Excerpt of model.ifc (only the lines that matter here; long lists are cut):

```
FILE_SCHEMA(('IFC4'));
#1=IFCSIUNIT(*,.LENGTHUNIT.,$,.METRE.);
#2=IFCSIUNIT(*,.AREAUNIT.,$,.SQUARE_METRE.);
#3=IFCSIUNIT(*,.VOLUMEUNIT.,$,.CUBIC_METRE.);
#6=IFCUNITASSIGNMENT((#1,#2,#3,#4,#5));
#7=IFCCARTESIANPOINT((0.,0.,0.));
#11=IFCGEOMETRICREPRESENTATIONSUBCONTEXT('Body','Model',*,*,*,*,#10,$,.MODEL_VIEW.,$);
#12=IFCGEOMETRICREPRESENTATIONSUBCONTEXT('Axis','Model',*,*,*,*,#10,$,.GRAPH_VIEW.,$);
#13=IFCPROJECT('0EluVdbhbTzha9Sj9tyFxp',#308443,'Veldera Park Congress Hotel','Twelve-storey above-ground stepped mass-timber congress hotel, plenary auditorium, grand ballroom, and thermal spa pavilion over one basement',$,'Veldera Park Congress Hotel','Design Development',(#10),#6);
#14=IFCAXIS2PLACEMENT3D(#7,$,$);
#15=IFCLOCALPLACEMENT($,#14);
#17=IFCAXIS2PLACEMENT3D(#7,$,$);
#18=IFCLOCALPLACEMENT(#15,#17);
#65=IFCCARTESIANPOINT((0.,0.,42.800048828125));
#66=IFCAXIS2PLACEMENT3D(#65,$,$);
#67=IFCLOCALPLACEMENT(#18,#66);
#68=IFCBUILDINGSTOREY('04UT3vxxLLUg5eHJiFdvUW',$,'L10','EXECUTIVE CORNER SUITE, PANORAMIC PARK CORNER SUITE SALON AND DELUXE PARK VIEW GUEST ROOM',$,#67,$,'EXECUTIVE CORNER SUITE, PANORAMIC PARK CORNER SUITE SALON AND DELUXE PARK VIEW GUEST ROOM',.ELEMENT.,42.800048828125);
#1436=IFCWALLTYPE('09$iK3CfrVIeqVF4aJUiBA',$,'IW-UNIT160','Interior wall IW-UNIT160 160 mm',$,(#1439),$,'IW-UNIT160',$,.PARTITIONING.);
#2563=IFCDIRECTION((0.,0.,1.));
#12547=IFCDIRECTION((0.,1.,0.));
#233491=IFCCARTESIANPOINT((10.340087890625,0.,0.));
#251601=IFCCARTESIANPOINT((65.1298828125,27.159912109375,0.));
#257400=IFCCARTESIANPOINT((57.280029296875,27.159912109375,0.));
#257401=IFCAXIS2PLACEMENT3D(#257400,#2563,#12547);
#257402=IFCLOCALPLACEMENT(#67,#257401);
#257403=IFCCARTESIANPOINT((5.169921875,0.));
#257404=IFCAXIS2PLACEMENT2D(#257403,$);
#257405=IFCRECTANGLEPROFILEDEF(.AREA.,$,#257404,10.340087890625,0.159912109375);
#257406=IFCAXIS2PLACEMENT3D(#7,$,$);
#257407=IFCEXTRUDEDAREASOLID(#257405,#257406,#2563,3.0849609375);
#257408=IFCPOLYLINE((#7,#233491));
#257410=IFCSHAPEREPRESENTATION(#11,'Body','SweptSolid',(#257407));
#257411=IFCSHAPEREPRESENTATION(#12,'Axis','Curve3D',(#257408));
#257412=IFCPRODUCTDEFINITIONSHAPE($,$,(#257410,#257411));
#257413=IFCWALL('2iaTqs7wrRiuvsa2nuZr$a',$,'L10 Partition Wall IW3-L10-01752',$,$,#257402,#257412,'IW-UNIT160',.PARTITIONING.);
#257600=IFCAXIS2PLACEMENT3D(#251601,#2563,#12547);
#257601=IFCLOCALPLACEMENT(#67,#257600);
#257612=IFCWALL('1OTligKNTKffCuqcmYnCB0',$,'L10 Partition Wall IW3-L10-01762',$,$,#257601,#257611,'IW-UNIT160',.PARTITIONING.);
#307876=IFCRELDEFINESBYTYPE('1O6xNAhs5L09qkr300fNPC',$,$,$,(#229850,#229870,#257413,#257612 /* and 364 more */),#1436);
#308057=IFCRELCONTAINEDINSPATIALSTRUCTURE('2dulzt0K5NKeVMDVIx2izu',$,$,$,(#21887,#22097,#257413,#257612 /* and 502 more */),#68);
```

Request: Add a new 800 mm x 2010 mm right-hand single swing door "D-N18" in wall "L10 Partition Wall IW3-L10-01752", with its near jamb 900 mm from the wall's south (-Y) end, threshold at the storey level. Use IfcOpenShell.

```python
import numpy as np
import ifcopenshell
import ifcopenshell.api.feature
import ifcopenshell.api.geometry
import ifcopenshell.api.root
import ifcopenshell.api.spatial
import ifcopenshell.geom
import ifcopenshell.util.element
import ifcopenshell.util.placement
import ifcopenshell.util.representation
import ifcopenshell.util.shape
import ifcopenshell.util.unit

model = ifcopenshell.open("model.ifc")
unit_scale = ifcopenshell.util.unit.calculate_unit_scale(model)
settings = ifcopenshell.geom.settings()


def volume(element):
    """Net volume in cubic metres, openings subtracted."""
    shape = ifcopenshell.geom.create_shape(settings, element)
    return ifcopenshell.util.shape.get_volume(shape.geometry)


wall = model.by_id(257413)
storey = ifcopenshell.util.element.get_container(wall, ifc_class="IfcBuildingStorey")
context = ifcopenshell.util.representation.get_context(model, "Model", "Body", "MODEL_VIEW")
before = volume(wall)

width, height, from_end, sill = 0.8, 2.01, 0.9, 0.0  # metres

# The wall runs along its own X axis, and the end named is its -X end.
wall_shape = ifcopenshell.geom.create_shape(settings, wall)
x, y, z = ifcopenshell.util.shape.get_vertices(wall_shape.geometry).T
start = x.min() + from_end
face, thickness = float(y.min()), float(y.max() - y.min())
wall_matrix = ifcopenshell.util.placement.get_local_placement(wall.ObjectPlacement)
level = ifcopenshell.util.placement.get_local_placement(storey.ObjectPlacement)[2, 3]


def in_wall(x, y):
    """Placement at x, y metres in the wall's axes, at sill height."""
    matrix = wall_matrix.copy()
    matrix[:, 3] = wall_matrix @ np.array([x / unit_scale, y / unit_scale, 0.0, 1.0])
    matrix[2, 3] = level + sill / unit_scale
    return matrix


# Opening: a box that overshoots both wall faces by 50 mm.
opening = ifcopenshell.api.root.create_entity(model, ifc_class="IfcOpeningElement", predefined_type="OPENING")
box = ifcopenshell.api.geometry.add_wall_representation(
    model, context=context, length=width, height=height, thickness=thickness + 0.1
)
ifcopenshell.api.geometry.assign_representation(model, product=opening, representation=box)
ifcopenshell.api.geometry.edit_object_placement(model, product=opening, matrix=in_wall(start, face - 0.05), is_si=False)
ifcopenshell.api.feature.add_feature(model, feature=opening, element=wall)

door = ifcopenshell.api.root.create_entity(model, ifc_class="IfcDoor", name="D-N18", predefined_type="DOOR")
door.OverallWidth, door.OverallHeight = width / unit_scale, height / unit_scale
door.OperationType = "SINGLE_SWING_RIGHT"
body = ifcopenshell.api.geometry.add_door_representation(
    model,
    context=context,
    overall_width=door.OverallWidth,
    overall_height=door.OverallHeight,
    operation_type="SINGLE_SWING_RIGHT",
    lining_properties={"LiningDepth": thickness / unit_scale, "ThresholdDepth": thickness / unit_scale},
)
ifcopenshell.api.geometry.assign_representation(model, product=door, representation=body)
ifcopenshell.api.spatial.assign_container(model, products=[door], relating_structure=storey)
ifcopenshell.api.feature.add_filling(model, opening=opening, element=door)

# The lining spans the wall, so the door starts at the wall face.
ifcopenshell.api.geometry.edit_object_placement(model, product=door, matrix=in_wall(start, face), is_si=False)

after = volume(wall)

print(f"wall volume {before:.3f} -> {after:.3f} m3")

model.write("model-out.ifc")
```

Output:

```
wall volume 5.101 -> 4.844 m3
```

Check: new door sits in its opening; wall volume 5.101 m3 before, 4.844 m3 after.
